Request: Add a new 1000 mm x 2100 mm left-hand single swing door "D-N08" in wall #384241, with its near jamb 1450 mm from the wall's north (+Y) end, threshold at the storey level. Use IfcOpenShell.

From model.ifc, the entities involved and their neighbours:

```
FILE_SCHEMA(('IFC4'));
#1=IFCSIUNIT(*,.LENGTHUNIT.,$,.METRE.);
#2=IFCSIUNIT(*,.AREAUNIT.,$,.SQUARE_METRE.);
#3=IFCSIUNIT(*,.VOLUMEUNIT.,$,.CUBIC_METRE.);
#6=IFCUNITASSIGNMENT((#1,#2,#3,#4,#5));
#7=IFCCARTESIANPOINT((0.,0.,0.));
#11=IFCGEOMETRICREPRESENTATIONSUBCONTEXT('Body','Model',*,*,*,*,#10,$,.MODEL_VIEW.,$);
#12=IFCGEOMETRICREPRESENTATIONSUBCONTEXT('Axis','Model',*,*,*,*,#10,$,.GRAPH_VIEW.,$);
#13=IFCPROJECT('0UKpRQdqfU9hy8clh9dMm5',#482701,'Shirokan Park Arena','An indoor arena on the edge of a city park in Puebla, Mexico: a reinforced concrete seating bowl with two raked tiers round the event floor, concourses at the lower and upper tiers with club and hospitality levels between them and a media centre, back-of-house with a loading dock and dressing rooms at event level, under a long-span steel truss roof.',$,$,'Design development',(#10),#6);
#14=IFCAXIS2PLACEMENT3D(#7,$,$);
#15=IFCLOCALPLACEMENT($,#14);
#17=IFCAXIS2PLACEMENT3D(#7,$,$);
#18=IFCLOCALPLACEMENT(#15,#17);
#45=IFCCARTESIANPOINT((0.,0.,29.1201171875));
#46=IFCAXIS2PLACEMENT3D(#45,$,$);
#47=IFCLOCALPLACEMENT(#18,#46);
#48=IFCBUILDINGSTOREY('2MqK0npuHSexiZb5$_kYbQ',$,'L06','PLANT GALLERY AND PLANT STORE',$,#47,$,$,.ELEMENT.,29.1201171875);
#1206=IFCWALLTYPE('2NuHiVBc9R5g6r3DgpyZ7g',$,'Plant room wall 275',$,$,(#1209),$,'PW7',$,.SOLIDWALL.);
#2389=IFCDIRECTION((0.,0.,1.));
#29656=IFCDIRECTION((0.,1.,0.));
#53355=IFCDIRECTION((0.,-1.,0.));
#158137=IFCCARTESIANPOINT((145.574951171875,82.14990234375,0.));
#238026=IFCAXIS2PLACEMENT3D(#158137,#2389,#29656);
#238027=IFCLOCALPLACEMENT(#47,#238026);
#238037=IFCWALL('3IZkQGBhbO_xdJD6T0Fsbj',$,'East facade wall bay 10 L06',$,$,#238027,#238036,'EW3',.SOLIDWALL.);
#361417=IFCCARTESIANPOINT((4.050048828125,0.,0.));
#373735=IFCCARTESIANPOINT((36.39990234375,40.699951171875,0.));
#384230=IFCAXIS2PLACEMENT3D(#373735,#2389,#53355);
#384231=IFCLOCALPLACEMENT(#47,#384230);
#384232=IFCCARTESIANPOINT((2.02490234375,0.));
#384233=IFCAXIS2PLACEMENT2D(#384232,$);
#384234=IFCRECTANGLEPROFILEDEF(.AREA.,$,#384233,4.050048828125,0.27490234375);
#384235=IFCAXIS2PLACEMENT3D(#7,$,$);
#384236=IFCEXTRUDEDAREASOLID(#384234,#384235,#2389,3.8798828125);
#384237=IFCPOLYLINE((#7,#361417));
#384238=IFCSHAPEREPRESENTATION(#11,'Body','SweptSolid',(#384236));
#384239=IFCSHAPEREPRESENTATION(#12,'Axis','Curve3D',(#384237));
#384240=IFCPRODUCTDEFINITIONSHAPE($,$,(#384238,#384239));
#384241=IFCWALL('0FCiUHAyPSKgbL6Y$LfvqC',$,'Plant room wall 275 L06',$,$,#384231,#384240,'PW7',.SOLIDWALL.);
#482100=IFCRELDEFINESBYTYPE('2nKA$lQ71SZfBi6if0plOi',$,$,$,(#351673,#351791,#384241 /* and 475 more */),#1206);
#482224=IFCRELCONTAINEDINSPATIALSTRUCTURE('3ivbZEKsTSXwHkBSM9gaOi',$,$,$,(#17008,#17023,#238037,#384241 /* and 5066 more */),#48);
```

```python
import numpy as np
import ifcopenshell
import ifcopenshell.api.feature
import ifcopenshell.api.geometry
import ifcopenshell.api.root
import ifcopenshell.api.spatial
import ifcopenshell.geom
import ifcopenshell.util.element
import ifcopenshell.util.placement
import ifcopenshell.util.representation
import ifcopenshell.util.shape
import ifcopenshell.util.unit

model = ifcopenshell.open("model.ifc")
unit_scale = ifcopenshell.util.unit.calculate_unit_scale(model)
settings = ifcopenshell.geom.settings()


def volume(element):
    """Net volume in cubic metres, openings subtracted."""
    shape = ifcopenshell.geom.create_shape(settings, element)
    return ifcopenshell.util.shape.get_volume(shape.geometry)


wall = model.by_guid("0FCiUHAyPSKgbL6Y$LfvqC")
storey = ifcopenshell.util.element.get_container(wall, ifc_class="IfcBuildingStorey")
context = ifcopenshell.util.representation.get_context(model, "Model", "Body", "MODEL_VIEW")
before = volume(wall)

width, height, from_end, sill = 1, 2.1, 1.45, 0.0  # metres

# The wall runs along its own X axis, and the end named is its -X end.
wall_shape = ifcopenshell.geom.create_shape(settings, wall)
x, y, z = ifcopenshell.util.shape.get_vertices(wall_shape.geometry).T
start = x.min() + from_end
face, thickness = float(y.min()), float(y.max() - y.min())
wall_matrix = ifcopenshell.util.placement.get_local_placement(wall.ObjectPlacement)
level = ifcopenshell.util.placement.get_local_placement(storey.ObjectPlacement)[2, 3]


def in_wall(x, y):
    """Placement at x, y metres in the wall's axes, at sill height."""
    matrix = wall_matrix.copy()
    matrix[:, 3] = wall_matrix @ np.array([x / unit_scale, y / unit_scale, 0.0, 1.0])
    matrix[2, 3] = level + sill / unit_scale
    return matrix


# Opening: a box that overshoots both wall faces by 50 mm.
opening = ifcopenshell.api.root.create_entity(model, ifc_class="IfcOpeningElement", predefined_type="OPENING")
box = ifcopenshell.api.geometry.add_wall_representation(
    model, context=context, length=width, height=height, thickness=thickness + 0.1
)
ifcopenshell.api.geometry.assign_representation(model, product=opening, representation=box)
ifcopenshell.api.geometry.edit_object_placement(model, product=opening, matrix=in_wall(start, face - 0.05), is_si=False)
ifcopenshell.api.feature.add_feature(model, feature=opening, element=wall)

door = ifcopenshell.api.root.create_entity(model, ifc_class="IfcDoor", name="D-N08", predefined_type="DOOR")
door.OverallWidth, door.OverallHeight = width / unit_scale, height / unit_scale
door.OperationType = "SINGLE_SWING_LEFT"
body = ifcopenshell.api.geometry.add_door_representation(
    model,
    context=context,
    overall_width=door.OverallWidth,
    overall_height=door.OverallHeight,
    operation_type="SINGLE_SWING_LEFT",
    lining_properties={"LiningDepth": thickness / unit_scale, "ThresholdDepth": thickness / unit_scale},
)
ifcopenshell.api.geometry.assign_representation(model, product=door, representation=body)
ifcopenshell.api.spatial.assign_container(model, products=[door], relating_structure=storey)
ifcopenshell.api.feature.add_filling(model, opening=opening, element=door)

# The lining spans the wall, so the door starts at the wall face.
ifcopenshell.api.geometry.edit_object_placement(model, product=door, matrix=in_wall(start, face), is_si=False)

after = volume(wall)

print(f"wall volume {before:.3f} -> {after:.3f} m3")

model.write("model-out.ifc")
```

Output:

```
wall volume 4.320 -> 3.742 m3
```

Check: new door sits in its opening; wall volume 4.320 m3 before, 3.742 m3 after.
